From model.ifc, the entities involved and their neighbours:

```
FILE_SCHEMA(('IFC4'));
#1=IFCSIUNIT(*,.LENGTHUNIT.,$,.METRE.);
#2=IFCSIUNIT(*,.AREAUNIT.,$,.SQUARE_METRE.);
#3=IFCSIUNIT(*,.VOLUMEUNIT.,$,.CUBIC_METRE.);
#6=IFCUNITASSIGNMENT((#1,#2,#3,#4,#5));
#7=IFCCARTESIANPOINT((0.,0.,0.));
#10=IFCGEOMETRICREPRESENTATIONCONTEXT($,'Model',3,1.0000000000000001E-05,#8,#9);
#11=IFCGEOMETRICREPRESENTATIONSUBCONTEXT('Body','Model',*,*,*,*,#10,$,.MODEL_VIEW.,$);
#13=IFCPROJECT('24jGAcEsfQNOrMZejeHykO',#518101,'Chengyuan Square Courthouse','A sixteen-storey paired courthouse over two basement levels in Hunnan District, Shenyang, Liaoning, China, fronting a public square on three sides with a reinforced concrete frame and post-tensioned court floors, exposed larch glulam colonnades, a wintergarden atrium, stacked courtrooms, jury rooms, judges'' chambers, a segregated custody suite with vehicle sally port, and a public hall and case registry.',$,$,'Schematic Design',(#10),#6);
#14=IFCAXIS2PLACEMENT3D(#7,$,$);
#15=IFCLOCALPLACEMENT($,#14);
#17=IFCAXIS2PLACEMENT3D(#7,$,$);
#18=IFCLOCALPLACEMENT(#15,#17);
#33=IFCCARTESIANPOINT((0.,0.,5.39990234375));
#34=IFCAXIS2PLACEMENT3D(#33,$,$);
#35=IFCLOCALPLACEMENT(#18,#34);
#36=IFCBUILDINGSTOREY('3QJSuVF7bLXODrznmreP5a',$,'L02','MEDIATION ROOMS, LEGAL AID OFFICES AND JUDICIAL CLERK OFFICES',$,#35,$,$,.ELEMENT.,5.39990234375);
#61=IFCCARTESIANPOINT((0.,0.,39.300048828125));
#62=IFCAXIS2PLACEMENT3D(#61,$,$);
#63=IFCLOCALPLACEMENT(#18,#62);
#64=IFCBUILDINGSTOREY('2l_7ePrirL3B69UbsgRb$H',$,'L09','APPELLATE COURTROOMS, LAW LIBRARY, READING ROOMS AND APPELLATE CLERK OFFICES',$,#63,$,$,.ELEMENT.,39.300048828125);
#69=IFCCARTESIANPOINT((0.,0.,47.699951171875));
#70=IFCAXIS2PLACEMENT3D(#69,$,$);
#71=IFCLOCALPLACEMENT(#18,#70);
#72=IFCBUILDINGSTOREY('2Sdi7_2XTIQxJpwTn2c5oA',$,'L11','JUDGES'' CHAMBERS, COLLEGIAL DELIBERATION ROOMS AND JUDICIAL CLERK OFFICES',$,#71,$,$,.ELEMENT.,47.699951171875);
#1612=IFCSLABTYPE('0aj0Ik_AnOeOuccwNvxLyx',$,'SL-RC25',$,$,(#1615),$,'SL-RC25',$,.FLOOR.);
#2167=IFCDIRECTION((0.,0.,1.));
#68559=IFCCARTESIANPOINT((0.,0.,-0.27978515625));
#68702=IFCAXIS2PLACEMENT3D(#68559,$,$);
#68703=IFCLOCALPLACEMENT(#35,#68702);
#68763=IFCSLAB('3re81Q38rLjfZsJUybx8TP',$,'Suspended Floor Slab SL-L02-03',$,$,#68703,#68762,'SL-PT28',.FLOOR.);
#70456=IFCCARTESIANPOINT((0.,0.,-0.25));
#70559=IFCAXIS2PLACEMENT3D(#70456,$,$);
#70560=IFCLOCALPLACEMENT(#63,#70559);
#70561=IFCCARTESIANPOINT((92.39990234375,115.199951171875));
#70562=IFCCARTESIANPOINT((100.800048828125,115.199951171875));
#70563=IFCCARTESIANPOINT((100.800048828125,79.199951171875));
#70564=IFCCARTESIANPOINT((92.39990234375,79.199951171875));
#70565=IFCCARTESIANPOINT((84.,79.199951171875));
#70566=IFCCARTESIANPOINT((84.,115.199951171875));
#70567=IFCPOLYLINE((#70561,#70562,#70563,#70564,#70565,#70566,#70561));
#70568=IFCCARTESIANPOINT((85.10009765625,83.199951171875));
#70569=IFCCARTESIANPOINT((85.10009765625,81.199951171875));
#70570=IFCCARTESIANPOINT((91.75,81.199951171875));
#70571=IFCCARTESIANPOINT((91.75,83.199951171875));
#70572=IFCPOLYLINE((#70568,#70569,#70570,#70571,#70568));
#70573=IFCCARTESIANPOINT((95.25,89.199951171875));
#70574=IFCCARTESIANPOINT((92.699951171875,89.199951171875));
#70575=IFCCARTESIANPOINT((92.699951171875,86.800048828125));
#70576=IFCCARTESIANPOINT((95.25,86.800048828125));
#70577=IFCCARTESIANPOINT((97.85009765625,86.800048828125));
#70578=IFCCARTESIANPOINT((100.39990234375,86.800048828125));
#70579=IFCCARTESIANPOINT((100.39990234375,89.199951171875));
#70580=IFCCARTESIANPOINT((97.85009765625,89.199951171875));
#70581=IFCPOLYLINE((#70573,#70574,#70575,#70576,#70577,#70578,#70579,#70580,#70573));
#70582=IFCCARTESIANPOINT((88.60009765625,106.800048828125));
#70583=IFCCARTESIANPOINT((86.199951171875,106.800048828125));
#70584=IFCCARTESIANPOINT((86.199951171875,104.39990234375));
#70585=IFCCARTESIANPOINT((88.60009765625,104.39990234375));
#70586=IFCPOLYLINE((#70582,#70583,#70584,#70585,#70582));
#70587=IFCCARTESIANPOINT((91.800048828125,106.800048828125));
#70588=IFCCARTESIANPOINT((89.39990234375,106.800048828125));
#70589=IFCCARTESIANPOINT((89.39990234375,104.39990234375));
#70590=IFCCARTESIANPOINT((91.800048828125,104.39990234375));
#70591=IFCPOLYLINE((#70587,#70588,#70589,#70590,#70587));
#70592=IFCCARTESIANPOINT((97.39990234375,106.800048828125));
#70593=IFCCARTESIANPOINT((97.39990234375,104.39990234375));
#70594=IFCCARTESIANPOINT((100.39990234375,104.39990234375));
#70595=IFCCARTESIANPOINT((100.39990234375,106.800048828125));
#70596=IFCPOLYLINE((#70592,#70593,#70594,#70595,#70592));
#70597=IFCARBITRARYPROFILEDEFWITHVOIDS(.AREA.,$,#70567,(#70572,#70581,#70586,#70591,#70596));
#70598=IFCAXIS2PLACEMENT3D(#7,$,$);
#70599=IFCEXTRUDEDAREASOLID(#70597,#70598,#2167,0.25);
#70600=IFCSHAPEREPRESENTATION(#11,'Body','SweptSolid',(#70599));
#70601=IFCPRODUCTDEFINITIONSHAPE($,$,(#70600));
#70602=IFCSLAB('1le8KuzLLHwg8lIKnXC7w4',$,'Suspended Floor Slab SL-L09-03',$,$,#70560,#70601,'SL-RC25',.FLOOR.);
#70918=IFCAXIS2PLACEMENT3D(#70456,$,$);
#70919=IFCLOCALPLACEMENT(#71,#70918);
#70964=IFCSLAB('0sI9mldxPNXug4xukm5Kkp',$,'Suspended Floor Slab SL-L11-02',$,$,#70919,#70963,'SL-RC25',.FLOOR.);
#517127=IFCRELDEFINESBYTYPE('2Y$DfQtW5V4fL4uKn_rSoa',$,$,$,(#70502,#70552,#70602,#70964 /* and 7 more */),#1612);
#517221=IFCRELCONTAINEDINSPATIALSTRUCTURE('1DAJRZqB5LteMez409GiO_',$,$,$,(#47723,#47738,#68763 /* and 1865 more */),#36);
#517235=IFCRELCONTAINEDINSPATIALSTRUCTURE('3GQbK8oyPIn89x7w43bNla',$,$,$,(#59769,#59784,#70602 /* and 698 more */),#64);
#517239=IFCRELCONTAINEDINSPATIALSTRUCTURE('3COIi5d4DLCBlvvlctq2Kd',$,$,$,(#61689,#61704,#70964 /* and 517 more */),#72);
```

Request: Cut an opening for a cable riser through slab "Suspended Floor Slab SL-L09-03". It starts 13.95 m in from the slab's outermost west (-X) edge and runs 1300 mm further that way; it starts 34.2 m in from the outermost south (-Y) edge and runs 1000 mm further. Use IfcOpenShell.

```python
import numpy as np
import ifcopenshell
import ifcopenshell.api.feature
import ifcopenshell.api.geometry
import ifcopenshell.api.root
import ifcopenshell.geom
import ifcopenshell.util.placement
import ifcopenshell.util.representation
import ifcopenshell.util.shape
import ifcopenshell.util.unit

model = ifcopenshell.open("model.ifc")
unit_scale = ifcopenshell.util.unit.calculate_unit_scale(model)
settings = ifcopenshell.geom.settings()


def volume(element):
    """Net volume in cubic metres, openings subtracted."""
    shape = ifcopenshell.geom.create_shape(settings, element)
    return ifcopenshell.util.shape.get_volume(shape.geometry)


slab = model.by_id(70602)
before = volume(slab)

# Extent in the slab's own axes, in metres. The edges named are its -X and -Y sides.
slab_shape = ifcopenshell.geom.create_shape(settings, slab)
vertices = ifcopenshell.util.shape.get_vertices(slab_shape.geometry)
x_min, y_min, bottom = vertices.min(axis=0)
top = vertices[:, 2].max()

opening = ifcopenshell.api.root.create_entity(model, ifc_class="IfcOpeningElement", name="Cable riser opening", predefined_type="OPENING")
context = ifcopenshell.util.representation.get_context(model, "Model", "Body", "MODEL_VIEW")
width, depth = 1.3, 1
outline = [(0.0, 0.0), (width, 0.0), (width, depth), (0.0, depth), (0.0, 0.0)]
# Overshoot both faces by 50 mm so the cut is clean.
shape = ifcopenshell.api.geometry.add_slab_representation(
    model, context=context, depth=top - bottom + 0.1, polyline=outline
)
ifcopenshell.api.geometry.assign_representation(model, product=opening, representation=shape)

matrix = ifcopenshell.util.placement.get_local_placement(slab.ObjectPlacement)
matrix[:, 3] = matrix @ np.append(np.array([x_min + 13.95, y_min + 34.2, bottom - 0.05]) / unit_scale, 1.0)
ifcopenshell.api.geometry.edit_object_placement(model, product=opening, matrix=matrix, is_si=False)
ifcopenshell.api.feature.add_feature(model, feature=opening, element=slab)

after = volume(slab)

print(f"slab volume {before:.3f} -> {after:.3f} m3")

model.write("model-out.ifc")
```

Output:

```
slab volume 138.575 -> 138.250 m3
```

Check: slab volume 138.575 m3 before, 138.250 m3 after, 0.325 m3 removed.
